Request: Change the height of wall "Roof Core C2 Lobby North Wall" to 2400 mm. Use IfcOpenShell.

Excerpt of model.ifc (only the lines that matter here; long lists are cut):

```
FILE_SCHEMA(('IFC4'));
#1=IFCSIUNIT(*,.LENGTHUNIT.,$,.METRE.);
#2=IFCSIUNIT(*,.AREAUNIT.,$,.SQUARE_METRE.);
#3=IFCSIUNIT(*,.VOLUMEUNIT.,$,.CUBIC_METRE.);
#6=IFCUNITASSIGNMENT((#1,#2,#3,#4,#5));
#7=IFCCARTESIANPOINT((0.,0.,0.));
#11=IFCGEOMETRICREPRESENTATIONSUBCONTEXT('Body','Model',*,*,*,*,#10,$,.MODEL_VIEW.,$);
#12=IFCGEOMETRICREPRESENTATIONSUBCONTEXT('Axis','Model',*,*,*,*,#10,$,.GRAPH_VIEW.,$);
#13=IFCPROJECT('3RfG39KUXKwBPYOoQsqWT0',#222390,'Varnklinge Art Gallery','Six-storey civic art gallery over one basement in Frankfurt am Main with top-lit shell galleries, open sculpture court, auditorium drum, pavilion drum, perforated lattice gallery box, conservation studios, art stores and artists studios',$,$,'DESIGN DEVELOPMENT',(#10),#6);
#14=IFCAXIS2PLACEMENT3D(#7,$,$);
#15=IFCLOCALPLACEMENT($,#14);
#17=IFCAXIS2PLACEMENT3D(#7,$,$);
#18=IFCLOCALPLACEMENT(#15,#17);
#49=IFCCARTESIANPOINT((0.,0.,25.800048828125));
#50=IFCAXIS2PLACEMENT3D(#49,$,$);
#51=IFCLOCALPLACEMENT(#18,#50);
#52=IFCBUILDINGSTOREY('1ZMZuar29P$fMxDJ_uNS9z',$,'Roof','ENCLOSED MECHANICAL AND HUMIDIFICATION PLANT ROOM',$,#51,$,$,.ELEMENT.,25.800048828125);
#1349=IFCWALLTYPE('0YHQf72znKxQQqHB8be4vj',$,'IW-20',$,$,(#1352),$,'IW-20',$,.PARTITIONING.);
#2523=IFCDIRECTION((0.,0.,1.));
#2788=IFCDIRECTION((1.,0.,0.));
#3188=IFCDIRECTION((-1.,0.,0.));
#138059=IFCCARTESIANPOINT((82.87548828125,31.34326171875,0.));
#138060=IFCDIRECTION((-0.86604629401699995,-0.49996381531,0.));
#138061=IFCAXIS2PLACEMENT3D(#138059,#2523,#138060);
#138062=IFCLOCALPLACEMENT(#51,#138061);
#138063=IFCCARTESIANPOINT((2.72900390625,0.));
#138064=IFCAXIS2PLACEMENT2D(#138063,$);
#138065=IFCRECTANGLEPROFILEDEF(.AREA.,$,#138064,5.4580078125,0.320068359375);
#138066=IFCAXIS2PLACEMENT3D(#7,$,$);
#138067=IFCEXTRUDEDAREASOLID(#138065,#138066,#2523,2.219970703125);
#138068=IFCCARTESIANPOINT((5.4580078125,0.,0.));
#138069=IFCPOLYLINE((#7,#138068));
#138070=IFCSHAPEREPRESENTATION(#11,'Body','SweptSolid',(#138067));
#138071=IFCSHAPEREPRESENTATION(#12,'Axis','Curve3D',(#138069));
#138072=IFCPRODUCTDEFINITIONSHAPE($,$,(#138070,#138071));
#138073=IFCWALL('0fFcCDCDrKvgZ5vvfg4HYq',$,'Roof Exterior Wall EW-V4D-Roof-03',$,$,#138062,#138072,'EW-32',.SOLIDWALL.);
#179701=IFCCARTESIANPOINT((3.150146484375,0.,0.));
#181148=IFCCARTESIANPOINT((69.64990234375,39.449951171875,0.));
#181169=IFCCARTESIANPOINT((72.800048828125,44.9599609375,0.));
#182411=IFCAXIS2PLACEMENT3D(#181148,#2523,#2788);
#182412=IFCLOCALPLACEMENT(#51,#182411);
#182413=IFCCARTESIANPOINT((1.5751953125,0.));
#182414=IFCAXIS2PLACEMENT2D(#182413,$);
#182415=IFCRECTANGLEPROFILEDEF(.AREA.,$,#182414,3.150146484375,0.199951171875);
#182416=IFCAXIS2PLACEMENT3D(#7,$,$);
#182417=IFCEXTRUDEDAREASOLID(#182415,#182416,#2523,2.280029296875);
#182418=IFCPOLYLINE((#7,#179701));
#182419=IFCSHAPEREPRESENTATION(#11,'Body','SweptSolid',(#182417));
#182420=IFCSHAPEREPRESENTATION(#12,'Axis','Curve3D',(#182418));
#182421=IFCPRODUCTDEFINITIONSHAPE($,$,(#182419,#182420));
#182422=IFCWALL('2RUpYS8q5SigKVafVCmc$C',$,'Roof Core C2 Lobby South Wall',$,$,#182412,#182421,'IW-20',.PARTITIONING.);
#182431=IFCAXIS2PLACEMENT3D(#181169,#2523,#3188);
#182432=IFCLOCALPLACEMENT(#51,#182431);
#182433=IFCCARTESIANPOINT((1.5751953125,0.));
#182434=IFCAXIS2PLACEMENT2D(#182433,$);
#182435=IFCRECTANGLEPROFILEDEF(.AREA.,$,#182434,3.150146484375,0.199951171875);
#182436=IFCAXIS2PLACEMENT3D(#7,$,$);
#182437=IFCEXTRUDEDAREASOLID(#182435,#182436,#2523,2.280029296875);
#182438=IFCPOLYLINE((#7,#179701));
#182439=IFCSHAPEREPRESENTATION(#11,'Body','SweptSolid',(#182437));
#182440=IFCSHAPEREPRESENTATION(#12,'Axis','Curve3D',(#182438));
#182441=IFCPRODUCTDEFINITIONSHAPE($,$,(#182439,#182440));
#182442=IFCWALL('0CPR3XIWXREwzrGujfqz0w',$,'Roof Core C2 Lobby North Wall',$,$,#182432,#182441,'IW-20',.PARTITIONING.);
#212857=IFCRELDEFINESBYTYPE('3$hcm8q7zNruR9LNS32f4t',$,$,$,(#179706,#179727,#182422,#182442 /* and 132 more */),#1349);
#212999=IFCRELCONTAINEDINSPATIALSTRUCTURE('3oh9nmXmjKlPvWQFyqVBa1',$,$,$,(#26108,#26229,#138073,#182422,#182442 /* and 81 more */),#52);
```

```python
import ifcopenshell
import ifcopenshell.geom
import ifcopenshell.util.representation
import ifcopenshell.util.shape
import ifcopenshell.util.unit

model = ifcopenshell.open("model.ifc")
unit_scale = ifcopenshell.util.unit.calculate_unit_scale(model)
settings = ifcopenshell.geom.settings()


def volume(element):
    """Net volume in cubic metres, openings subtracted."""
    shape = ifcopenshell.geom.create_shape(settings, element)
    return ifcopenshell.util.shape.get_volume(shape.geometry)


wall = model.by_guid("0CPR3XIWXREwzrGujfqz0w")
before = volume(wall)

body = ifcopenshell.util.representation.get_representation(wall, "Model", "Body")
solid = body.Items[0]
old_height = solid.Depth
solid.Depth = 2.4 / unit_scale
after = volume(wall)

print(f"height {old_height:g} -> {solid.Depth:g}, volume {before:.3f} -> {after:.3f} m3")

model.write("model_edited.ifc")
```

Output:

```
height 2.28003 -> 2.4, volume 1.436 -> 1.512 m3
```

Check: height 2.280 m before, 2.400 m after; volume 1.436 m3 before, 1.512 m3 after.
